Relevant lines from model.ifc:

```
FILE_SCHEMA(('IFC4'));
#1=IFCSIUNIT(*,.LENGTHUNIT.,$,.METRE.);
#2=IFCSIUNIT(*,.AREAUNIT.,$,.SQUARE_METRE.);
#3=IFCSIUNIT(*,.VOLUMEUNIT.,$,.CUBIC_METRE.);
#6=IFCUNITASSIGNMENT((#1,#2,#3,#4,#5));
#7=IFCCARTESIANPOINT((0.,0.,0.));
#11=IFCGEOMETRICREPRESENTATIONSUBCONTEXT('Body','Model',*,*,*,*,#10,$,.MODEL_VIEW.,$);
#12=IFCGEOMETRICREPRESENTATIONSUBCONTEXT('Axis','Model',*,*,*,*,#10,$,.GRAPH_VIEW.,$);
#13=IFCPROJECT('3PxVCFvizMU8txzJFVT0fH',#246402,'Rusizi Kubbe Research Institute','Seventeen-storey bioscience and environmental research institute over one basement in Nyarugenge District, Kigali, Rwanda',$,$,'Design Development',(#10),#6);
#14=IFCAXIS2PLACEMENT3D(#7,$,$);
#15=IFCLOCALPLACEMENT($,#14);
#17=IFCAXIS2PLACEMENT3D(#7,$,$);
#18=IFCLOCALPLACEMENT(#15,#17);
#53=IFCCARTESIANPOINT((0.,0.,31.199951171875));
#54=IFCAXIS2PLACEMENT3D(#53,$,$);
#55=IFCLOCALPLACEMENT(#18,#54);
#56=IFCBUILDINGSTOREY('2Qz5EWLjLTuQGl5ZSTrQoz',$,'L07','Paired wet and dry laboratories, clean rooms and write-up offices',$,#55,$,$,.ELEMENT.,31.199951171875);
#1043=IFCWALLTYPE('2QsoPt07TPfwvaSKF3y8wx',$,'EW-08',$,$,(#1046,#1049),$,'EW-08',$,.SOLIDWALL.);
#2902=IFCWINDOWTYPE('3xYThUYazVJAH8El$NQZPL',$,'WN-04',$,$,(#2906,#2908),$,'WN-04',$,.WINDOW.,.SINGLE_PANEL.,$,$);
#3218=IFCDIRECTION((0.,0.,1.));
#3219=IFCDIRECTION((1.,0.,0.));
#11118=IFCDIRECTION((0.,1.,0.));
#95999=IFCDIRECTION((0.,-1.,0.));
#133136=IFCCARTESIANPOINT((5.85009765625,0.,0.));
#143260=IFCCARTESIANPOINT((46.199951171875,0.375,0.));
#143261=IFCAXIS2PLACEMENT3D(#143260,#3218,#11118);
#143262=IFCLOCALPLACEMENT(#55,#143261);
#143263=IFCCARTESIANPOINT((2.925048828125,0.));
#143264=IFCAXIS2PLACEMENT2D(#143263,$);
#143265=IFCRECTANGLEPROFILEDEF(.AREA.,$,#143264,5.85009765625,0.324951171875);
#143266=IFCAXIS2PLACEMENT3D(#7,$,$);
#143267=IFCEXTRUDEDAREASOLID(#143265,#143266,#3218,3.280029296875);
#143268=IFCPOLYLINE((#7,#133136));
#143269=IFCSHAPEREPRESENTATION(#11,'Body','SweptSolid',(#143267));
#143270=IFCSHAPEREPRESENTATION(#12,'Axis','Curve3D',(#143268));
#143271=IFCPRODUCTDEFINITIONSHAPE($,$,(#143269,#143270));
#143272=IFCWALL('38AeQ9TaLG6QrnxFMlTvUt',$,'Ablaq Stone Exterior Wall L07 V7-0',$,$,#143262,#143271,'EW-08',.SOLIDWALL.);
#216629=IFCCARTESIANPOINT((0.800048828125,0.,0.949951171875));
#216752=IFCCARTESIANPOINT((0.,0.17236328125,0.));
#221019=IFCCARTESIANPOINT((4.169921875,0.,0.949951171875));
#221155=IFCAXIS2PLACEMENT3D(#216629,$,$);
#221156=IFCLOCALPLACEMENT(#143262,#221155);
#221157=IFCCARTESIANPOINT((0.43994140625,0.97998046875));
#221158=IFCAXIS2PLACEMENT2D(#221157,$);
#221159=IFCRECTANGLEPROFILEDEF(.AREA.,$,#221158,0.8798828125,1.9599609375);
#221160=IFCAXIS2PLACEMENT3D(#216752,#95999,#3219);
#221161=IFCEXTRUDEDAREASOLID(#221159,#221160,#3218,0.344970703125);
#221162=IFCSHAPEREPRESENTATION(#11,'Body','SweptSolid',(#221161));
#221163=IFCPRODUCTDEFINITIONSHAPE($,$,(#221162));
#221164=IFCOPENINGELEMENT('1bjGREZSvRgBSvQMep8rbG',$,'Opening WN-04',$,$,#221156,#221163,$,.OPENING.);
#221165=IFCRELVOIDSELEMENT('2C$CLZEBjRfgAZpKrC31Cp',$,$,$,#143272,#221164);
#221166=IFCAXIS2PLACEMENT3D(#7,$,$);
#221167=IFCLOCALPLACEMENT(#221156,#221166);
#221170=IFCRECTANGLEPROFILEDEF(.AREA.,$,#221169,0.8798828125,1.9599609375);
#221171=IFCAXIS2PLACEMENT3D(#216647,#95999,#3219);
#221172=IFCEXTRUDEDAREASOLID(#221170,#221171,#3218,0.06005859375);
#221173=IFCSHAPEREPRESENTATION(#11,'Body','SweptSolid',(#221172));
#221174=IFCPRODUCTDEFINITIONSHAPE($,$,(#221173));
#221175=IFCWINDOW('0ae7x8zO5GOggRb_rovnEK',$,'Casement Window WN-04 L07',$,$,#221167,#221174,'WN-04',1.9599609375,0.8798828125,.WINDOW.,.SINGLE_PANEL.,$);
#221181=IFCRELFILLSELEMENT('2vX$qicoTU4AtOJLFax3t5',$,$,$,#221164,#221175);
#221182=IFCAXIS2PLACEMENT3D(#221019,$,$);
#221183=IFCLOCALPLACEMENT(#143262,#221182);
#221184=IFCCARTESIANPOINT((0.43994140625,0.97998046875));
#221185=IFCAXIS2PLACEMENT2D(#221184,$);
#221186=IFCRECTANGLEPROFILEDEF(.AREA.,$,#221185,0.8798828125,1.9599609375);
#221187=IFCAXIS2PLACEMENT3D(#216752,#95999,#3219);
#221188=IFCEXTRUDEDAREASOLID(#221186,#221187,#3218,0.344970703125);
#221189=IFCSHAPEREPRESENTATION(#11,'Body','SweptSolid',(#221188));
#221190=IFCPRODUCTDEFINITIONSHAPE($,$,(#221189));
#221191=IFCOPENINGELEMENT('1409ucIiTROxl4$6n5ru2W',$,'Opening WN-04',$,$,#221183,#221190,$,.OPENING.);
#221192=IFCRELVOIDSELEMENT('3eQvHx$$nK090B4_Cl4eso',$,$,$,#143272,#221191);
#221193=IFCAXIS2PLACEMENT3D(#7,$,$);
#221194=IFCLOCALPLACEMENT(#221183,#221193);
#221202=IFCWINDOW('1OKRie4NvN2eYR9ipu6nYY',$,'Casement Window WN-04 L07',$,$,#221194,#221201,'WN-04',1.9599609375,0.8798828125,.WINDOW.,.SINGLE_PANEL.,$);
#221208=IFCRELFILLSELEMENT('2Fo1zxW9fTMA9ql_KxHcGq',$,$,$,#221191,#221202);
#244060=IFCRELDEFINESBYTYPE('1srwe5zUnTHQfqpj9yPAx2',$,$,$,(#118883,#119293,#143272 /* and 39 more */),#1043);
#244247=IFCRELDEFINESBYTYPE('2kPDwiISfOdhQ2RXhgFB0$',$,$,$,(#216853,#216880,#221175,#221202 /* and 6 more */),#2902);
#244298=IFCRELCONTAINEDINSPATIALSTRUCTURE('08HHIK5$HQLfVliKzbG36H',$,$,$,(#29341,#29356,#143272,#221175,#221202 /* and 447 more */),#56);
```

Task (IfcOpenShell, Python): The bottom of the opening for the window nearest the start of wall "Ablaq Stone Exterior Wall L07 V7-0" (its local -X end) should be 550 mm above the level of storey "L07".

```python
import numpy as np
import ifcopenshell
import ifcopenshell.api.geometry
import ifcopenshell.geom
import ifcopenshell.util.element
import ifcopenshell.util.placement
import ifcopenshell.util.shape
import ifcopenshell.util.unit

model = ifcopenshell.open("model.ifc")
unit_scale = ifcopenshell.util.unit.calculate_unit_scale(model)

window = model.by_guid("0ae7x8zO5GOggRb_rovnEK")
opening = window.FillsVoids[0].RelatingOpeningElement
storey = ifcopenshell.util.element.get_container(window, ifc_class="IfcBuildingStorey")
level = ifcopenshell.util.placement.get_local_placement(storey.ObjectPlacement)[2, 3]

# The opening's origin need not be at the sill, so measure its lowest point.
shape = ifcopenshell.geom.create_shape(ifcopenshell.geom.settings(), opening)
bottom = ifcopenshell.util.shape.get_shape_bottom_elevation(shape, shape.geometry) / unit_scale
dz = level + 0.55 - bottom

shift = np.array([0.0, 0.0, dz])
# The window is placed relative to its opening, so it follows when the opening moves.
matrix = ifcopenshell.util.placement.get_local_placement(opening.ObjectPlacement)
matrix[:3, 3] += shift
ifcopenshell.api.geometry.edit_object_placement(
    model, product=opening, matrix=matrix, is_si=False, should_transform_children=True
)

print(f"moved by {dz * unit_scale:+.3f} m")

model.write("model_updated.ifc")
```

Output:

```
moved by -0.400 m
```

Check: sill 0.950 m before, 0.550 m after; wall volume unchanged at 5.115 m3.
